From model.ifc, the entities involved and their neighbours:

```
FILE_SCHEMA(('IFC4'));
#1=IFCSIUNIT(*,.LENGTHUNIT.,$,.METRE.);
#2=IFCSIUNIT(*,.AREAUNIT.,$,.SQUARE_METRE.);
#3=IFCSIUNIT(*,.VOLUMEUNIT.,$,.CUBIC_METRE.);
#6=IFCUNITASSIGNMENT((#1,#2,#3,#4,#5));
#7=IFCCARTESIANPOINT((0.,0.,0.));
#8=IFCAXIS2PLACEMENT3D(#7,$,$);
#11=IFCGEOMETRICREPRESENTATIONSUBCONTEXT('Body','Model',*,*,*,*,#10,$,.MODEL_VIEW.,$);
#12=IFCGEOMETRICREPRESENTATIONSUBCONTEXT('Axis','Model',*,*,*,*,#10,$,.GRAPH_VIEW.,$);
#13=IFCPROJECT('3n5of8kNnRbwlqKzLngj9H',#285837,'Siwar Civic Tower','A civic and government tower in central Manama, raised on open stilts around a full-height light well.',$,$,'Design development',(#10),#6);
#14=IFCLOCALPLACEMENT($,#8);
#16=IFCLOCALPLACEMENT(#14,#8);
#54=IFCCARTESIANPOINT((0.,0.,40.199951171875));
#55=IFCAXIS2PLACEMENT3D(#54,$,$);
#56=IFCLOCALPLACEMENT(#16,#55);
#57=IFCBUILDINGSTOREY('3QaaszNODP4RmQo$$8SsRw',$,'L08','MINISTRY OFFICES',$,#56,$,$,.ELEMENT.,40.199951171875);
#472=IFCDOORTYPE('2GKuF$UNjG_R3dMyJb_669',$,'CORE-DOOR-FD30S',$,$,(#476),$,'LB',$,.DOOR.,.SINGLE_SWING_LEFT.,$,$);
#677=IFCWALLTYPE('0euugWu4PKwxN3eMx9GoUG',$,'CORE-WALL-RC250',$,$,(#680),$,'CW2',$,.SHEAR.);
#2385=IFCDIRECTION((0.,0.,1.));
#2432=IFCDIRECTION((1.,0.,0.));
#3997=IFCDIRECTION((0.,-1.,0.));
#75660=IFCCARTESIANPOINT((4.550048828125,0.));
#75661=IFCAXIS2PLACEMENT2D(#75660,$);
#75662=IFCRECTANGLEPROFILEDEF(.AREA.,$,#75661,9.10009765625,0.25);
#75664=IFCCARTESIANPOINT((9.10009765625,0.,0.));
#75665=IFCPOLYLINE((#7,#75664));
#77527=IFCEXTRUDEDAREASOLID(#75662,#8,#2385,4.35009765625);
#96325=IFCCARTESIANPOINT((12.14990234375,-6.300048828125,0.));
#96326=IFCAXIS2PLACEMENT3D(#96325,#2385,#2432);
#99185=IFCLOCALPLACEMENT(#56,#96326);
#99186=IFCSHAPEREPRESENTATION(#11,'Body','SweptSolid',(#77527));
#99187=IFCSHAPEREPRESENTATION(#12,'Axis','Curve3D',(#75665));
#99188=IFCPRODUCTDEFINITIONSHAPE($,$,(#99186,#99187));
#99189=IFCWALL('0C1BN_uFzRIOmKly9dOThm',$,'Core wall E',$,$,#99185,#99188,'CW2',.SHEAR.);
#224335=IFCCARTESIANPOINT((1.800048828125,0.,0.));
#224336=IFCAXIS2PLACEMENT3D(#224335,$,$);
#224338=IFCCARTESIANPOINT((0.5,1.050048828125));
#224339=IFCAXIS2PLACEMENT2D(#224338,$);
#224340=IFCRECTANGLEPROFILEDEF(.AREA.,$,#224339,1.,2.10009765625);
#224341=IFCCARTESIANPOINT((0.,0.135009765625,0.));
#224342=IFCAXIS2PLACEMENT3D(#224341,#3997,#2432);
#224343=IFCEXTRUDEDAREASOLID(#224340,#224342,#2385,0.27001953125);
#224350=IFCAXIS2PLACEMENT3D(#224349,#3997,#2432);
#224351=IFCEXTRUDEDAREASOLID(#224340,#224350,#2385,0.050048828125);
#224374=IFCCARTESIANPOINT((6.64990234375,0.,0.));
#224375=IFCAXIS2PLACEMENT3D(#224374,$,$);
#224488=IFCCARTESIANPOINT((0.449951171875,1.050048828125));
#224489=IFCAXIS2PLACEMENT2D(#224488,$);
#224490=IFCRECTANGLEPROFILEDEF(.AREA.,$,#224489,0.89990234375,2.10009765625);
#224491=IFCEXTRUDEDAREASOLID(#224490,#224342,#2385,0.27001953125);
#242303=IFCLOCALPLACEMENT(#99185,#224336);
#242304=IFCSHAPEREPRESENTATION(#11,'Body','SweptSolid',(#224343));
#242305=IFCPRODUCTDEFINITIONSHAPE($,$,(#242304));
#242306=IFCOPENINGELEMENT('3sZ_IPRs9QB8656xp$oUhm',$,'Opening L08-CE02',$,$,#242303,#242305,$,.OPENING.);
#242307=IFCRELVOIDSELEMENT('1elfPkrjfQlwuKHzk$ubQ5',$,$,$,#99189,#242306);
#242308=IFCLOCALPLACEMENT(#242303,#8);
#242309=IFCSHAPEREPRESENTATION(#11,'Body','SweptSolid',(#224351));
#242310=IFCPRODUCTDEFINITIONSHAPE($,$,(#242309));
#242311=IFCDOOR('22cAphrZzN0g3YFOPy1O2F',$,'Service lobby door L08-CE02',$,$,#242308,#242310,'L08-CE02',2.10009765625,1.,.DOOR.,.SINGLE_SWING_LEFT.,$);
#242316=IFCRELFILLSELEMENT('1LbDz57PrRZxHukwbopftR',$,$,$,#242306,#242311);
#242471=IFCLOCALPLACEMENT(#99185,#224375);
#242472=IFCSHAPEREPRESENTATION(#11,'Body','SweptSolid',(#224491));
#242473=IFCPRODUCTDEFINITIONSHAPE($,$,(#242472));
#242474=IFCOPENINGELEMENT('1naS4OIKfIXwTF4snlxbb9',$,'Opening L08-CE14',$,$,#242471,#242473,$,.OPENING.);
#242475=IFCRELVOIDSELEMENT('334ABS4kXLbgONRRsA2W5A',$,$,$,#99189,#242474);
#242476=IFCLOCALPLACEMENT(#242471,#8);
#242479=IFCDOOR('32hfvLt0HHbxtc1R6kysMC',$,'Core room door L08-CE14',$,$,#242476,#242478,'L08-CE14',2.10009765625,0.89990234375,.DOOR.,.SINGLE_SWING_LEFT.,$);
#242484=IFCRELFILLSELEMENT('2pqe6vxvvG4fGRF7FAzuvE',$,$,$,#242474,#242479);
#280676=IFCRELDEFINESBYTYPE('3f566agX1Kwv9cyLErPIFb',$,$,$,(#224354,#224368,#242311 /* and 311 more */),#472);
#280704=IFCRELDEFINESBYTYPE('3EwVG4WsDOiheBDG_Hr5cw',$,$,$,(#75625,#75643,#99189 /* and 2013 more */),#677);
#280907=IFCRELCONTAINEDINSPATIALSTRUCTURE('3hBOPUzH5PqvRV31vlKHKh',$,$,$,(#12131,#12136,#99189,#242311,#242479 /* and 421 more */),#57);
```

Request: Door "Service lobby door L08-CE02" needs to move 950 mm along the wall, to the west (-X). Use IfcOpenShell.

```python
import ifcopenshell
import ifcopenshell.api.geometry
import ifcopenshell.util.placement

model = ifcopenshell.open("model.ifc")

door = model.by_id(242311)
opening = door.FillsVoids[0].RelatingOpeningElement
wall = opening.VoidsElements[0].RelatingBuildingElement

wall_matrix = ifcopenshell.util.placement.get_local_placement(wall.ObjectPlacement)
shift = wall_matrix[:3, 0] * -0.95
before = ifcopenshell.util.placement.get_local_placement(door.ObjectPlacement)[:3, 3].copy()

# The door is placed relative to its opening, so it follows when the opening moves.
matrix = ifcopenshell.util.placement.get_local_placement(opening.ObjectPlacement)
matrix[:3, 3] += shift
ifcopenshell.api.geometry.edit_object_placement(
    model, product=opening, matrix=matrix, is_si=False, should_transform_children=True
)

after = ifcopenshell.util.placement.get_local_placement(door.ObjectPlacement)[:3, 3]
print("door moved by", (after - before).round(3) + 0.0)

model.write("model_edited.ifc")
```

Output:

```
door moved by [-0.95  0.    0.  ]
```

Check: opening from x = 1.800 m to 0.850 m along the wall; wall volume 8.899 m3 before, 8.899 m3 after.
